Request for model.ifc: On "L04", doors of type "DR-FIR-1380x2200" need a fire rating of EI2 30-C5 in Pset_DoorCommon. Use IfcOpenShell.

First a look at what the model holds.

```python
import ifcopenshell
import ifcopenshell.util.element

model = ifcopenshell.open("model.ifc")
print(model.schema)
storey = next(s for s in model.by_type("IfcBuildingStorey") if s.Name == "L04")
doors = [e for e in ifcopenshell.util.element.get_decomposition(storey) if e.is_a("IfcDoor")]
seen = {}
for e in doors:
    element_type = ifcopenshell.util.element.get_type(e)
    key = (element_type.Name if element_type != e and element_type else None, ifcopenshell.util.element.get_pset(e, "Pset_DoorCommon", "FireRating"))
    seen[key] = seen.get(key, 0) + 1
for (name, value), count in sorted(seen.items(), key=str):
    print(count, "x", name, "|", value)
```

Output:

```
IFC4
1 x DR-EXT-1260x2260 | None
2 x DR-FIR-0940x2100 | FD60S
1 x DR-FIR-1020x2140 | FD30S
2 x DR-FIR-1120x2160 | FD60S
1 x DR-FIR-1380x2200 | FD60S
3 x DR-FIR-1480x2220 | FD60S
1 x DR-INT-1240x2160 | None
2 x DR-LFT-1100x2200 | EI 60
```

```python
import ifcopenshell
import ifcopenshell.api.pset
import ifcopenshell.util.element

model = ifcopenshell.open("model.ifc")

storey = next(s for s in model.by_type("IfcBuildingStorey") if s.Name == "L04")
doors = [e for e in ifcopenshell.util.element.get_decomposition(storey) if e.is_a("IfcDoor")]

count = 0
for e in doors:
    element_type = ifcopenshell.util.element.get_type(e)
    if element_type in (None, e) or element_type.Name != "DR-FIR-1380x2200":
        continue
    # add_pset returns the element's existing set when there is one.
    pset = ifcopenshell.api.pset.add_pset(model, product=e, name="Pset_DoorCommon")
    ifcopenshell.api.pset.edit_pset(model, pset=pset, properties={"FireRating": "EI2 30-C5"})
    count += 1

print(count, "doors updated")

model.write("model_rev.ifc")
```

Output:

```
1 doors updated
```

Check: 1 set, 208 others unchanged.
